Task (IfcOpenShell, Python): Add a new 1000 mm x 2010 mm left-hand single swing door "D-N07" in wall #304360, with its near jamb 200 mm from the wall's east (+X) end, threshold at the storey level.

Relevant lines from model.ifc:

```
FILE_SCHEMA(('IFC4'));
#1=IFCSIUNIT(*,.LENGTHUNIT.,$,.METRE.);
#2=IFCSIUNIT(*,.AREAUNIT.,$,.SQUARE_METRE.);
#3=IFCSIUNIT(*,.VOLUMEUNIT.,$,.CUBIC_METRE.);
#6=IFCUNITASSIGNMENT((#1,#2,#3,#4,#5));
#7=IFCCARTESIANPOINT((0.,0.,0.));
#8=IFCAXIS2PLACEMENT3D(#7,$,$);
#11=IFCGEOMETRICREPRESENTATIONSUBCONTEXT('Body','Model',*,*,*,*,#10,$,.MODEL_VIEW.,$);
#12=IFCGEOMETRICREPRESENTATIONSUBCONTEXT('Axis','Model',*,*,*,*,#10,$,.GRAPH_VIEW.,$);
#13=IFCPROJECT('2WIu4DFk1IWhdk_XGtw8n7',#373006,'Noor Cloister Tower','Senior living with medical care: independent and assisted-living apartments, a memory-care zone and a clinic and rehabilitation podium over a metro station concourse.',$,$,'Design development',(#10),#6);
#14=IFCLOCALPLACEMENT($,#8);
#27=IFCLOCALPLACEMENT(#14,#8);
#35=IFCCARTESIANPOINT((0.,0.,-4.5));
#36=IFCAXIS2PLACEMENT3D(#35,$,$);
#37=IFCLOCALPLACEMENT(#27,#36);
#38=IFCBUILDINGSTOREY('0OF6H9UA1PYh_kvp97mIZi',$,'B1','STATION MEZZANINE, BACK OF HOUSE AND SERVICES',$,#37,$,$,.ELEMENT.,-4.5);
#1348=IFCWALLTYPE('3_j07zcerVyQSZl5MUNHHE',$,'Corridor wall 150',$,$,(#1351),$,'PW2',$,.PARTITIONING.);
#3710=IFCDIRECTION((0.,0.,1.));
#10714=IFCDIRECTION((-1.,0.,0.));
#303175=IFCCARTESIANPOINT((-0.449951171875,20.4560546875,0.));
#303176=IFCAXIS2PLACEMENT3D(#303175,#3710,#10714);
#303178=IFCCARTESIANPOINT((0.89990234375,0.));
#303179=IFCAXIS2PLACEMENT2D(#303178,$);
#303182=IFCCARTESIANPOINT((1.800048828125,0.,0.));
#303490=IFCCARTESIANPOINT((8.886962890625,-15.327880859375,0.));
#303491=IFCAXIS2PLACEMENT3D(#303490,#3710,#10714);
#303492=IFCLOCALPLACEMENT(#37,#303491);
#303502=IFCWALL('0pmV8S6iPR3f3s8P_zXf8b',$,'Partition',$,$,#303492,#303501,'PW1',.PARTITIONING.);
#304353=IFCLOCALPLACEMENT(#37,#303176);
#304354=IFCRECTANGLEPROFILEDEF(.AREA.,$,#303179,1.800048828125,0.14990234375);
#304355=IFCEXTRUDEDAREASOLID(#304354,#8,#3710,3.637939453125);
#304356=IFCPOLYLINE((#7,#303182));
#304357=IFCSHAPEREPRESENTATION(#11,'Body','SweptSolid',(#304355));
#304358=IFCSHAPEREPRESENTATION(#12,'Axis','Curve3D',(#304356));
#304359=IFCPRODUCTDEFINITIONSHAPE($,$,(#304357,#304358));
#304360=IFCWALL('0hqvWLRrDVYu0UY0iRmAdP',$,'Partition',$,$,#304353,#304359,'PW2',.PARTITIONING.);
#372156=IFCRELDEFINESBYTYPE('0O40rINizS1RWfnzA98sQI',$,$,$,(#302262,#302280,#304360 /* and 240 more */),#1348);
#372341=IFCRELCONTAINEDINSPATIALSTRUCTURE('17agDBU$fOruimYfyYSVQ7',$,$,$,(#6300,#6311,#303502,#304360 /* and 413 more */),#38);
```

```python
import numpy as np
import ifcopenshell
import ifcopenshell.api.feature
import ifcopenshell.api.geometry
import ifcopenshell.api.root
import ifcopenshell.api.spatial
import ifcopenshell.geom
import ifcopenshell.util.element
import ifcopenshell.util.placement
import ifcopenshell.util.representation
import ifcopenshell.util.shape
import ifcopenshell.util.unit

model = ifcopenshell.open("model.ifc")
unit_scale = ifcopenshell.util.unit.calculate_unit_scale(model)
settings = ifcopenshell.geom.settings()


def volume(element):
    """Net volume in cubic metres, openings subtracted."""
    shape = ifcopenshell.geom.create_shape(settings, element)
    return ifcopenshell.util.shape.get_volume(shape.geometry)


wall = model.by_guid("0hqvWLRrDVYu0UY0iRmAdP")
storey = ifcopenshell.util.element.get_container(wall, ifc_class="IfcBuildingStorey")
context = ifcopenshell.util.representation.get_context(model, "Model", "Body", "MODEL_VIEW")
before = volume(wall)

width, height, from_end, sill = 1, 2.01, 0.2, 0.0  # metres

# The wall runs along its own X axis, and the end named is its -X end.
wall_shape = ifcopenshell.geom.create_shape(settings, wall)
x, y, z = ifcopenshell.util.shape.get_vertices(wall_shape.geometry).T
start = x.min() + from_end
face, thickness = float(y.min()), float(y.max() - y.min())
wall_matrix = ifcopenshell.util.placement.get_local_placement(wall.ObjectPlacement)
level = ifcopenshell.util.placement.get_local_placement(storey.ObjectPlacement)[2, 3]


def in_wall(x, y):
    """Placement at x, y metres in the wall's axes, at sill height."""
    matrix = wall_matrix.copy()
    matrix[:, 3] = wall_matrix @ np.array([x / unit_scale, y / unit_scale, 0.0, 1.0])
    matrix[2, 3] = level + sill / unit_scale
    return matrix


# Opening: a box that overshoots both wall faces by 50 mm.
opening = ifcopenshell.api.root.create_entity(model, ifc_class="IfcOpeningElement", predefined_type="OPENING")
box = ifcopenshell.api.geometry.add_wall_representation(
    model, context=context, length=width, height=height, thickness=thickness + 0.1
)
ifcopenshell.api.geometry.assign_representation(model, product=opening, representation=box)
ifcopenshell.api.geometry.edit_object_placement(model, product=opening, matrix=in_wall(start, face - 0.05), is_si=False)
ifcopenshell.api.feature.add_feature(model, feature=opening, element=wall)

door = ifcopenshell.api.root.create_entity(model, ifc_class="IfcDoor", name="D-N07", predefined_type="DOOR")
door.OverallWidth, door.OverallHeight = width / unit_scale, height / unit_scale
door.OperationType = "SINGLE_SWING_LEFT"
body = ifcopenshell.api.geometry.add_door_representation(
    model,
    context=context,
    overall_width=door.OverallWidth,
    overall_height=door.OverallHeight,
    operation_type="SINGLE_SWING_LEFT",
    lining_properties={"LiningDepth": thickness / unit_scale, "ThresholdDepth": thickness / unit_scale},
)
ifcopenshell.api.geometry.assign_representation(model, product=door, representation=body)
ifcopenshell.api.spatial.assign_container(model, products=[door], relating_structure=storey)
ifcopenshell.api.feature.add_filling(model, opening=opening, element=door)

# The lining spans the wall, so the door starts at the wall face.
ifcopenshell.api.geometry.edit_object_placement(model, product=door, matrix=in_wall(start, face), is_si=False)

after = volume(wall)

print(f"wall volume {before:.3f} -> {after:.3f} m3")

model.write("model_updated.ifc")
```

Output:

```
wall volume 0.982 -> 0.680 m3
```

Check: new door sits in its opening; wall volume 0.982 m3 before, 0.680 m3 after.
